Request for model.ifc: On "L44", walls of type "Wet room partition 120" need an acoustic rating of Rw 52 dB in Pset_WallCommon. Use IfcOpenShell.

First a look at what the model holds.

```python
import ifcopenshell
import ifcopenshell.util.element

model = ifcopenshell.open("model.ifc")
print(model.schema)
storey = next(s for s in model.by_type("IfcBuildingStorey") if s.Name == "L44")
walls = [e for e in ifcopenshell.util.element.get_decomposition(storey) if e.is_a("IfcWall")]
seen = {}
for e in walls:
    element_type = ifcopenshell.util.element.get_type(e)
    key = (element_type.Name if element_type != e and element_type else None, ifcopenshell.util.element.get_pset(e, "Pset_WallCommon", "AcousticRating"))
    seen[key] = seen.get(key, 0) + 1
for (name, value), count in sorted(seen.items(), key=str):
    print(count, "x", name, "|", value)
```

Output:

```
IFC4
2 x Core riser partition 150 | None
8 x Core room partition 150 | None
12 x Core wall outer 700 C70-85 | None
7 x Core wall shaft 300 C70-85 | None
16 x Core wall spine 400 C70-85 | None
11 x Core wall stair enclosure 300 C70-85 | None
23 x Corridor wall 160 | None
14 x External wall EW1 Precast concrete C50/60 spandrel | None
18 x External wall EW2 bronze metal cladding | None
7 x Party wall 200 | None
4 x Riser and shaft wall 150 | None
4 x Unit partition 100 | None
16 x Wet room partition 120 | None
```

```python
import ifcopenshell
import ifcopenshell.api.pset
import ifcopenshell.util.element

model = ifcopenshell.open("model.ifc")

storey = next(s for s in model.by_type("IfcBuildingStorey") if s.Name == "L44")
walls = [e for e in ifcopenshell.util.element.get_decomposition(storey) if e.is_a("IfcWall")]

count = 0
for e in walls:
    element_type = ifcopenshell.util.element.get_type(e)
    if element_type in (None, e) or element_type.Name != "Wet room partition 120":
        continue
    found = ifcopenshell.util.element.get_pset(e, "Pset_WallCommon", should_inherit=False)
    if found:
        pset = model.by_id(found["id"])
        if len(ifcopenshell.util.element.get_elements_by_pset(pset)) > 1:
            pset = ifcopenshell.api.pset.unshare_pset(model, products=[e], pset=pset)[0]
    else:
        pset = ifcopenshell.api.pset.add_pset(model, product=e, name="Pset_WallCommon")
    ifcopenshell.api.pset.edit_pset(model, pset=pset, properties={"AcousticRating": "Rw 52 dB"})
    count += 1

print(count, "walls updated")

model.write("model_rev.ifc")
```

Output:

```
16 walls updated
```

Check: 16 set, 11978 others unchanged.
